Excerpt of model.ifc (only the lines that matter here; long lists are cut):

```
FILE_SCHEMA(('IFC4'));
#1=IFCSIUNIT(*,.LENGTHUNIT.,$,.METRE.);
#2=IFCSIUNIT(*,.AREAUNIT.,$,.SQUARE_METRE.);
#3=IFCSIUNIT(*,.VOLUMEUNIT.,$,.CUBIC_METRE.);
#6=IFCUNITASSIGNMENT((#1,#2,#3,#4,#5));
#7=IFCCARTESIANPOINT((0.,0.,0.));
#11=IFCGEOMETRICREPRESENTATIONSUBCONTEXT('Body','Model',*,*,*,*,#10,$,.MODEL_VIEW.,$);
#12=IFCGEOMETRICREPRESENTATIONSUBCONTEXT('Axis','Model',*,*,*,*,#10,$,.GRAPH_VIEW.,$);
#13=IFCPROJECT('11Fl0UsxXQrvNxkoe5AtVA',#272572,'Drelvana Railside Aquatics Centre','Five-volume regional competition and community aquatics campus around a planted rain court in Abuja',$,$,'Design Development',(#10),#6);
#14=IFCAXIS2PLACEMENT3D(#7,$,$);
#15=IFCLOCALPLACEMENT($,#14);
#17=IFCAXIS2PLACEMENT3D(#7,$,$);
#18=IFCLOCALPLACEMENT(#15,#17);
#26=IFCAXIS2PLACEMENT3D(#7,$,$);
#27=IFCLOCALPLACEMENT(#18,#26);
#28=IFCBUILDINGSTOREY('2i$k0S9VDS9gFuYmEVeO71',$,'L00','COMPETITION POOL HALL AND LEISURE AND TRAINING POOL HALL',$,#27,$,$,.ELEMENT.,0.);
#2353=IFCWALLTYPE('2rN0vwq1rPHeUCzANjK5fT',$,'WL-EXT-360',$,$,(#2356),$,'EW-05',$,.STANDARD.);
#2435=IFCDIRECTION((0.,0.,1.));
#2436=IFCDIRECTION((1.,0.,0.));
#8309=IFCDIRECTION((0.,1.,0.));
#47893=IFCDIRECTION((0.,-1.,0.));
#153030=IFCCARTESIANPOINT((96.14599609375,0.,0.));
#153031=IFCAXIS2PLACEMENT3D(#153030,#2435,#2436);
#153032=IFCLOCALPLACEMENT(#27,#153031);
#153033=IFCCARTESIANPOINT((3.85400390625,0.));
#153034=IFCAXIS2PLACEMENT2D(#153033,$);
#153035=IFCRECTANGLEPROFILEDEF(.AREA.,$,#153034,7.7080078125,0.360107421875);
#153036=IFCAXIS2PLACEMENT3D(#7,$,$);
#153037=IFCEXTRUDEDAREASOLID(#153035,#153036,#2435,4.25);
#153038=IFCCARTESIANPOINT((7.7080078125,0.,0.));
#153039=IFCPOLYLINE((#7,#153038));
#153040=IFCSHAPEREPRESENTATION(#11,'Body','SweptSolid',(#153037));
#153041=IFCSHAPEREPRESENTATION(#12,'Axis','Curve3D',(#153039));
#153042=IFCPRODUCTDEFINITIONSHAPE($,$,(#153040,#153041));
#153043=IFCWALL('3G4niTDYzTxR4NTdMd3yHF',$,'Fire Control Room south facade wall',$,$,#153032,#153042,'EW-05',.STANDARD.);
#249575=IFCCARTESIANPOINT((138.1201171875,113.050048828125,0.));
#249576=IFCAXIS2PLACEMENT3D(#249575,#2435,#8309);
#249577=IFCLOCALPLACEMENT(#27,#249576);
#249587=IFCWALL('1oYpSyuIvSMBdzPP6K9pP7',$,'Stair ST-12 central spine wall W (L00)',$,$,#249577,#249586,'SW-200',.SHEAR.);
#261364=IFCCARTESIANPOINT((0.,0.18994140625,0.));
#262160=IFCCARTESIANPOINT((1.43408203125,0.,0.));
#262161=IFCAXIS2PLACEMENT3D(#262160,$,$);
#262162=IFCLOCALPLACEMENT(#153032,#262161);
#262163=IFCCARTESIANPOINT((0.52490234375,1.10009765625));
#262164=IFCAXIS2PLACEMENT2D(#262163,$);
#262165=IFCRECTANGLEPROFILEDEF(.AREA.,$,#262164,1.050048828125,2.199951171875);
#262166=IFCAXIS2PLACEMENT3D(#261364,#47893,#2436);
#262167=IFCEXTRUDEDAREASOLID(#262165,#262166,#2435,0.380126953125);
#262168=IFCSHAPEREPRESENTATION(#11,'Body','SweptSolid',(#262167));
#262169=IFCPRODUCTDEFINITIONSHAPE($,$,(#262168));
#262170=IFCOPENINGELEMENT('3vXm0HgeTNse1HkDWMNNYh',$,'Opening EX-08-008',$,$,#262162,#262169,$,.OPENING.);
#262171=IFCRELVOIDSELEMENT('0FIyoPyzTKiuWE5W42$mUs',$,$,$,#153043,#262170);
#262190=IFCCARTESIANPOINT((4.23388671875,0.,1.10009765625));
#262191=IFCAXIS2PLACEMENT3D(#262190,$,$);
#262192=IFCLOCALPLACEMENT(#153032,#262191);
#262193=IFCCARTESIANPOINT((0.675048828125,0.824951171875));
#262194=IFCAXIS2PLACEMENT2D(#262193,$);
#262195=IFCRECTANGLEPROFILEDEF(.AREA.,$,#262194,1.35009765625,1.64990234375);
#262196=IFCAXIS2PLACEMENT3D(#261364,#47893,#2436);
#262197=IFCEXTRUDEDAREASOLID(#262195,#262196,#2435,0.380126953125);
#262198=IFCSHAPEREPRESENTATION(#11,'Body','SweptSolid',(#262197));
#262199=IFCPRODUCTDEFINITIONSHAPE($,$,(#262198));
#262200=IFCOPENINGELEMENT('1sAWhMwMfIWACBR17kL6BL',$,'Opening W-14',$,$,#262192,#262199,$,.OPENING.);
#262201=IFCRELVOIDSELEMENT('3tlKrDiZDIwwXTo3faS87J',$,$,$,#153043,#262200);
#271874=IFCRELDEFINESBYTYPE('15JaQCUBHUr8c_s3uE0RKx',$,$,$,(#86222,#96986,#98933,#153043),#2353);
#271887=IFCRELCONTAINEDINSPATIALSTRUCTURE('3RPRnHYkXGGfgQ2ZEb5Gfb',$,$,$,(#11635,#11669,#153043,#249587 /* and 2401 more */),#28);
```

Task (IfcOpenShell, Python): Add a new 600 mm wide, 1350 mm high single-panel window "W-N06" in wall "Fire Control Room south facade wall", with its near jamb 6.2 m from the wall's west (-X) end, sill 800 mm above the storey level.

```python
import numpy as np
import ifcopenshell
import ifcopenshell.api.feature
import ifcopenshell.api.geometry
import ifcopenshell.api.root
import ifcopenshell.api.spatial
import ifcopenshell.geom
import ifcopenshell.util.element
import ifcopenshell.util.placement
import ifcopenshell.util.representation
import ifcopenshell.util.shape
import ifcopenshell.util.unit

model = ifcopenshell.open("model.ifc")
unit_scale = ifcopenshell.util.unit.calculate_unit_scale(model)
settings = ifcopenshell.geom.settings()


def volume(element):
    """Net volume in cubic metres, openings subtracted."""
    shape = ifcopenshell.geom.create_shape(settings, element)
    return ifcopenshell.util.shape.get_volume(shape.geometry)


wall = model.by_id(153043)
storey = ifcopenshell.util.element.get_container(wall, ifc_class="IfcBuildingStorey")
context = ifcopenshell.util.representation.get_context(model, "Model", "Body", "MODEL_VIEW")
before = volume(wall)

width, height, from_end, sill = 0.6, 1.35, 6.2, 0.8  # metres

# The wall runs along its own X axis, and the end named is its -X end.
wall_shape = ifcopenshell.geom.create_shape(settings, wall)
x, y, z = ifcopenshell.util.shape.get_vertices(wall_shape.geometry).T
start = x.min() + from_end
face, thickness = float(y.min()), float(y.max() - y.min())
wall_matrix = ifcopenshell.util.placement.get_local_placement(wall.ObjectPlacement)
level = ifcopenshell.util.placement.get_local_placement(storey.ObjectPlacement)[2, 3]


def in_wall(x, y):
    """Placement at x, y metres in the wall's axes, at sill height."""
    matrix = wall_matrix.copy()
    matrix[:, 3] = wall_matrix @ np.array([x / unit_scale, y / unit_scale, 0.0, 1.0])
    matrix[2, 3] = level + sill / unit_scale
    return matrix


# Opening: a box that overshoots both wall faces by 50 mm.
opening = ifcopenshell.api.root.create_entity(model, ifc_class="IfcOpeningElement", predefined_type="OPENING")
box = ifcopenshell.api.geometry.add_wall_representation(
    model, context=context, length=width, height=height, thickness=thickness + 0.1
)
ifcopenshell.api.geometry.assign_representation(model, product=opening, representation=box)
ifcopenshell.api.geometry.edit_object_placement(model, product=opening, matrix=in_wall(start, face - 0.05), is_si=False)
ifcopenshell.api.feature.add_feature(model, feature=opening, element=wall)

window = ifcopenshell.api.root.create_entity(model, ifc_class="IfcWindow", name="W-N06", predefined_type="WINDOW")
window.OverallWidth, window.OverallHeight = width / unit_scale, height / unit_scale
window.PartitioningType = "SINGLE_PANEL"
body = ifcopenshell.api.geometry.add_window_representation(
    model,
    context=context,
    overall_width=window.OverallWidth,
    overall_height=window.OverallHeight,
    partition_type="SINGLE_PANEL",
)
ifcopenshell.api.geometry.assign_representation(model, product=window, representation=body)
ifcopenshell.api.spatial.assign_container(model, products=[window], relating_structure=storey)
ifcopenshell.api.feature.add_filling(model, opening=opening, element=window)

# Centre the window in the wall's thickness.
ifcopenshell.api.geometry.edit_object_placement(model, product=window, matrix=in_wall(start, face), is_si=False)
window_shape = ifcopenshell.geom.create_shape(settings, window)
depth = ifcopenshell.util.shape.get_vertices(window_shape.geometry)[:, 1]
offset = face + thickness / 2 - (depth.min() + depth.max()) / 2
ifcopenshell.api.geometry.edit_object_placement(model, product=window, matrix=in_wall(start, offset), is_si=False)

after = volume(wall)

print(f"wall volume {before:.3f} -> {after:.3f} m3")

model.write("model_v2.ifc")
```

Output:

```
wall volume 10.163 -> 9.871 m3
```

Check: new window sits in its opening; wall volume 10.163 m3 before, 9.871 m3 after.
